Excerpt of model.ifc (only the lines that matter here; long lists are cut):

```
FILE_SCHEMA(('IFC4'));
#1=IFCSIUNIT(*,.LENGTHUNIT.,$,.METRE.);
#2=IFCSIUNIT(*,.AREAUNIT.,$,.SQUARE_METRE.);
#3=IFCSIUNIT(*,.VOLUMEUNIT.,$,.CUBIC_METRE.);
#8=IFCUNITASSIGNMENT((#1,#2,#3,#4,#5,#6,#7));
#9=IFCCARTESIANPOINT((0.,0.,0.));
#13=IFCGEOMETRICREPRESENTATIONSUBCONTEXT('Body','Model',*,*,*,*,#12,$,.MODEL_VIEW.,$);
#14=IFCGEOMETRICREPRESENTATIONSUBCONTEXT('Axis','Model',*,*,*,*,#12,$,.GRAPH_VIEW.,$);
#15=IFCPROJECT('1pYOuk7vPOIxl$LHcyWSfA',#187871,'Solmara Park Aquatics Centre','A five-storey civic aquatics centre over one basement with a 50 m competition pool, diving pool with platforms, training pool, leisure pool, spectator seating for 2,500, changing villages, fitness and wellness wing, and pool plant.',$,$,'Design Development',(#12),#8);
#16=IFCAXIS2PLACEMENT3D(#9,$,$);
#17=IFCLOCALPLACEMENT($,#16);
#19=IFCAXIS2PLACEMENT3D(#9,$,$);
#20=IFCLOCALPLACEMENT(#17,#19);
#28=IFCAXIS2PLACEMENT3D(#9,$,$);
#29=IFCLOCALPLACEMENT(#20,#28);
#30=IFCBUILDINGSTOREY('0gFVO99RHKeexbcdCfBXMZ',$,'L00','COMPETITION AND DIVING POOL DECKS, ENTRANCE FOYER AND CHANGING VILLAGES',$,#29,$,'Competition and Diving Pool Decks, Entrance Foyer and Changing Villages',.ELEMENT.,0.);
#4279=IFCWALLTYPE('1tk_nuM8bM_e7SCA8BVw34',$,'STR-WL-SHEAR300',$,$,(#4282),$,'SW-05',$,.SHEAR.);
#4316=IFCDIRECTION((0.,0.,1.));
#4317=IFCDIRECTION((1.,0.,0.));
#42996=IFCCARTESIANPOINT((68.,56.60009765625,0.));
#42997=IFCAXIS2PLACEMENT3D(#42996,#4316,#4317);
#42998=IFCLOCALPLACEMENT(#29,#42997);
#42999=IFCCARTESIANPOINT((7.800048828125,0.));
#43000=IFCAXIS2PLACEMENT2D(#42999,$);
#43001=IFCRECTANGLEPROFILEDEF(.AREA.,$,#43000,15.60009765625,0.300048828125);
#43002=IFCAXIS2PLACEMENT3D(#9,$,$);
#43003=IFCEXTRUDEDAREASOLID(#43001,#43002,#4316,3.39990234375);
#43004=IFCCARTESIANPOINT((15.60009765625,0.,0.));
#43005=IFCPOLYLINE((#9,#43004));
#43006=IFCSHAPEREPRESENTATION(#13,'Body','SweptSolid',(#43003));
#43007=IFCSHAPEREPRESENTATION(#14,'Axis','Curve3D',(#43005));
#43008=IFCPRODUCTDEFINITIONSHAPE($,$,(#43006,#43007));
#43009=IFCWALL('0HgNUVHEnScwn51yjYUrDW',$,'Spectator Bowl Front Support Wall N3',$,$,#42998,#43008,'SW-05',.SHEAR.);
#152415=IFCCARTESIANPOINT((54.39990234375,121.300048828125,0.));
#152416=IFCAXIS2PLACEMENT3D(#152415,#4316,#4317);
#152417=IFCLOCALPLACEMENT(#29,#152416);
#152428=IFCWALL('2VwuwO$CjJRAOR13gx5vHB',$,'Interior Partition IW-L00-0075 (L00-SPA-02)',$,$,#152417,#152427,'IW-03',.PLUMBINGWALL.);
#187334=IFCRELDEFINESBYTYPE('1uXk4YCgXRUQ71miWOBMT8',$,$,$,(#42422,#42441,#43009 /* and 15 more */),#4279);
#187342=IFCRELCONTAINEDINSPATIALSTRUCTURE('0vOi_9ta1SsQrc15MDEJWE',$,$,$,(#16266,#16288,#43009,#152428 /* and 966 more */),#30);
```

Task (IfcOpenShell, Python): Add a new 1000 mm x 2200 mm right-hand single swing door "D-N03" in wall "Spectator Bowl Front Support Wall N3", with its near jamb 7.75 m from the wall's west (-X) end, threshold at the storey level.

```python
import numpy as np
import ifcopenshell
import ifcopenshell.api.feature
import ifcopenshell.api.geometry
import ifcopenshell.api.root
import ifcopenshell.api.spatial
import ifcopenshell.geom
import ifcopenshell.util.element
import ifcopenshell.util.placement
import ifcopenshell.util.representation
import ifcopenshell.util.shape
import ifcopenshell.util.unit

model = ifcopenshell.open("model.ifc")
unit_scale = ifcopenshell.util.unit.calculate_unit_scale(model)
settings = ifcopenshell.geom.settings()


def volume(element):
    """Net volume in cubic metres, openings subtracted."""
    shape = ifcopenshell.geom.create_shape(settings, element)
    return ifcopenshell.util.shape.get_volume(shape.geometry)


wall = model.by_guid("0HgNUVHEnScwn51yjYUrDW")
storey = ifcopenshell.util.element.get_container(wall, ifc_class="IfcBuildingStorey")
context = ifcopenshell.util.representation.get_context(model, "Model", "Body", "MODEL_VIEW")
before = volume(wall)

width, height, from_end, sill = 1, 2.2, 7.75, 0.0  # metres

# The wall runs along its own X axis, and the end named is its -X end.
wall_shape = ifcopenshell.geom.create_shape(settings, wall)
x, y, z = ifcopenshell.util.shape.get_vertices(wall_shape.geometry).T
start = x.min() + from_end
face, thickness = float(y.min()), float(y.max() - y.min())
wall_matrix = ifcopenshell.util.placement.get_local_placement(wall.ObjectPlacement)
level = ifcopenshell.util.placement.get_local_placement(storey.ObjectPlacement)[2, 3]


def in_wall(x, y):
    """Placement at x, y metres in the wall's axes, at sill height."""
    matrix = wall_matrix.copy()
    matrix[:, 3] = wall_matrix @ np.array([x / unit_scale, y / unit_scale, 0.0, 1.0])
    matrix[2, 3] = level + sill / unit_scale
    return matrix


# Opening: a box that overshoots both wall faces by 50 mm.
opening = ifcopenshell.api.root.create_entity(model, ifc_class="IfcOpeningElement", predefined_type="OPENING")
box = ifcopenshell.api.geometry.add_wall_representation(
    model, context=context, length=width, height=height, thickness=thickness + 0.1
)
ifcopenshell.api.geometry.assign_representation(model, product=opening, representation=box)
ifcopenshell.api.geometry.edit_object_placement(model, product=opening, matrix=in_wall(start, face - 0.05), is_si=False)
ifcopenshell.api.feature.add_feature(model, feature=opening, element=wall)

door = ifcopenshell.api.root.create_entity(model, ifc_class="IfcDoor", name="D-N03", predefined_type="DOOR")
door.OverallWidth, door.OverallHeight = width / unit_scale, height / unit_scale
door.OperationType = "SINGLE_SWING_RIGHT"
body = ifcopenshell.api.geometry.add_door_representation(
    model,
    context=context,
    overall_width=door.OverallWidth,
    overall_height=door.OverallHeight,
    operation_type="SINGLE_SWING_RIGHT",
    lining_properties={"LiningDepth": thickness / unit_scale, "ThresholdDepth": thickness / unit_scale},
)
ifcopenshell.api.geometry.assign_representation(model, product=door, representation=body)
ifcopenshell.api.spatial.assign_container(model, products=[door], relating_structure=storey)
ifcopenshell.api.feature.add_filling(model, opening=opening, element=door)

# The lining spans the wall, so the door starts at the wall face.
ifcopenshell.api.geometry.edit_object_placement(model, product=door, matrix=in_wall(start, face), is_si=False)

after = volume(wall)

print(f"wall volume {before:.3f} -> {after:.3f} m3")

model.write("model_updated.ifc")
```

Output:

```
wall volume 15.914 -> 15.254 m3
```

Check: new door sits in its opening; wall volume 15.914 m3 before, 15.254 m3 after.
